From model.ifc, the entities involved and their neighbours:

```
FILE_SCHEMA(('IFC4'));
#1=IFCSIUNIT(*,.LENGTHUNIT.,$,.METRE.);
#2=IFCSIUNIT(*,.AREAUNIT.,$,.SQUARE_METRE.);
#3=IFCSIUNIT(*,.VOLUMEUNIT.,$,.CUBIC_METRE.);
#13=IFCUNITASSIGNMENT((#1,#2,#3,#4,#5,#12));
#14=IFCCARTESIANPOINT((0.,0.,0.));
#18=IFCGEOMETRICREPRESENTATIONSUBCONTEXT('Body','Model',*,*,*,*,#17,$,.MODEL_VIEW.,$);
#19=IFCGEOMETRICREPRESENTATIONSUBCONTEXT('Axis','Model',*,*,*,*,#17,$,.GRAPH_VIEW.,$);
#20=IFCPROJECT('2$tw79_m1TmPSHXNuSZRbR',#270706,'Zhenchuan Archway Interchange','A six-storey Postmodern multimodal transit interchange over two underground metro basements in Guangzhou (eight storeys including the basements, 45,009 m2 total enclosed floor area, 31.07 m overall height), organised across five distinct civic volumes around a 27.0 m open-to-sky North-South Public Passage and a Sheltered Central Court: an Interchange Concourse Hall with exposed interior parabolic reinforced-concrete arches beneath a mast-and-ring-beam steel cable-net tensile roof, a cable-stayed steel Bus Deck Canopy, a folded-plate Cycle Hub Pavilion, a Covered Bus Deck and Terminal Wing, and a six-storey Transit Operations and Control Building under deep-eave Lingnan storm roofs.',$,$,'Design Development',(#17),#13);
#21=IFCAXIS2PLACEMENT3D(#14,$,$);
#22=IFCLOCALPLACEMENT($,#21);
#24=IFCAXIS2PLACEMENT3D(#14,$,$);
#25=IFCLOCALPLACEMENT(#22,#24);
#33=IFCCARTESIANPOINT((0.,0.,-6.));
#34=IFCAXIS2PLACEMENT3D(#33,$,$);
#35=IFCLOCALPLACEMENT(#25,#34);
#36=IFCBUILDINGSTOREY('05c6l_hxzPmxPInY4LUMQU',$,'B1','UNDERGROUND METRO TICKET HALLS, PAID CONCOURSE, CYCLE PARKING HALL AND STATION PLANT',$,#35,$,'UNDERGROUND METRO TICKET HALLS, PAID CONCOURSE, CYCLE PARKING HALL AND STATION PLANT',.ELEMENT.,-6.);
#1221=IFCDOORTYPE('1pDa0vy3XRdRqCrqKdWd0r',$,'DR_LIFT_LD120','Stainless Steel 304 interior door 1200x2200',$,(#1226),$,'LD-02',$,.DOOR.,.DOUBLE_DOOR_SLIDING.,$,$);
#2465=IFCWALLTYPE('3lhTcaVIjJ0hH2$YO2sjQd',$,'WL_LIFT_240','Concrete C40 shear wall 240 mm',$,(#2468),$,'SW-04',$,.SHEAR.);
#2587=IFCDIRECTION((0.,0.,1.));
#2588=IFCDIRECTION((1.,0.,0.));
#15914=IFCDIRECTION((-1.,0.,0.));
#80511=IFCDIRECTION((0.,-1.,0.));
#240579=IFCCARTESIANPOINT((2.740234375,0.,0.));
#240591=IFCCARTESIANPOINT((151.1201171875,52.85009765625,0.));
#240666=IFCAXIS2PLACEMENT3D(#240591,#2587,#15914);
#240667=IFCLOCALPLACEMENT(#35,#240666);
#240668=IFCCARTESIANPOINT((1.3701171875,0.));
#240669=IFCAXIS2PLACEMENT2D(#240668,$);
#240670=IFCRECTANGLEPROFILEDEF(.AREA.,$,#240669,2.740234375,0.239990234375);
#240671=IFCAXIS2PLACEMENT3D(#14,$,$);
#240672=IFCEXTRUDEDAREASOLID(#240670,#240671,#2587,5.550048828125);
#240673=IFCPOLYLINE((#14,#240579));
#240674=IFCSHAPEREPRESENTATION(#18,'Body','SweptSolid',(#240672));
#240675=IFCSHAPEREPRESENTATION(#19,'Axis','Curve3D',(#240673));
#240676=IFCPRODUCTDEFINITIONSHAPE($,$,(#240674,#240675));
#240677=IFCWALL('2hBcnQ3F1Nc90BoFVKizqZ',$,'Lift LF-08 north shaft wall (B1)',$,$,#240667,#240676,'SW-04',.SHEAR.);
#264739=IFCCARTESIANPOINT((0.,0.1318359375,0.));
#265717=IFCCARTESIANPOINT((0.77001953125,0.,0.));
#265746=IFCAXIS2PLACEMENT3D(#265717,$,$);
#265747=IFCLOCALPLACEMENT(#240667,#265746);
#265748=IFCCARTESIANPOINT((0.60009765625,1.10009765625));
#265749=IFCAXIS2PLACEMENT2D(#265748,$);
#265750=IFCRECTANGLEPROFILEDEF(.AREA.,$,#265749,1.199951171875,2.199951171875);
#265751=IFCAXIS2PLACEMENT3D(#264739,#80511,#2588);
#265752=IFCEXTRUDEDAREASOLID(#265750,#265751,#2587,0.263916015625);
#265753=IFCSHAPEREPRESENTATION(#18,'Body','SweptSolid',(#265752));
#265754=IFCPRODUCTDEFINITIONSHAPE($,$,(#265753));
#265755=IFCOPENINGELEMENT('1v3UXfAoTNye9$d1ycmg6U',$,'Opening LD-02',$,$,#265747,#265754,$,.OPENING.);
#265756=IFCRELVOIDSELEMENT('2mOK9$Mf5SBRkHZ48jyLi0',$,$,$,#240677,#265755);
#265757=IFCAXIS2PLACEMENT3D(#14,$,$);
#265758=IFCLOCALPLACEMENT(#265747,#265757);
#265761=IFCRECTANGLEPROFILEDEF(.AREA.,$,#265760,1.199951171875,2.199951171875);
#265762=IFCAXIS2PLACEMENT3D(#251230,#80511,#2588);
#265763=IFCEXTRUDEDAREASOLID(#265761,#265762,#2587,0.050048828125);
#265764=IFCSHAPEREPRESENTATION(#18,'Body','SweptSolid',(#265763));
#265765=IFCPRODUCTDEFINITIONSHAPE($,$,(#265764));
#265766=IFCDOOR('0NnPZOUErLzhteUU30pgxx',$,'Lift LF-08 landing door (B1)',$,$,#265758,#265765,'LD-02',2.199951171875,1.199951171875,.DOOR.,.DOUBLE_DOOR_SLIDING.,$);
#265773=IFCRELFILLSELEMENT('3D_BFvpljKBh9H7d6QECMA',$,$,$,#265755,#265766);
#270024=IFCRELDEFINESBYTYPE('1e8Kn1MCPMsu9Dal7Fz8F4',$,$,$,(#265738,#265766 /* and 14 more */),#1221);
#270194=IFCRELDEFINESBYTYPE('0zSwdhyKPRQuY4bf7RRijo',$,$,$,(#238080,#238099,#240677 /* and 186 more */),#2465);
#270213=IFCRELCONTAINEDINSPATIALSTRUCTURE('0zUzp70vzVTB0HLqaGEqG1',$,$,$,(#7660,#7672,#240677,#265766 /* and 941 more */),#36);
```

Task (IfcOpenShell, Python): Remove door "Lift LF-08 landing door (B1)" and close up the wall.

```python
import ifcopenshell
import ifcopenshell.api.feature
import ifcopenshell.api.root
import ifcopenshell.geom
import ifcopenshell.util.shape

model = ifcopenshell.open("model.ifc")
settings = ifcopenshell.geom.settings()


def volume(element):
    """Net volume in cubic metres, openings subtracted."""
    shape = ifcopenshell.geom.create_shape(settings, element)
    return ifcopenshell.util.shape.get_volume(shape.geometry)


door = model.by_id(265766)
opening = door.FillsVoids[0].RelatingOpeningElement
wall = opening.VoidsElements[0].RelatingBuildingElement
before = volume(wall)

ifcopenshell.api.root.remove_product(model, product=door)
ifcopenshell.api.feature.remove_feature(model, feature=opening)

after = volume(wall)

print(f"wall volume {before:.3f} -> {after:.3f} m3")

model.write("model_updated.ifc")
```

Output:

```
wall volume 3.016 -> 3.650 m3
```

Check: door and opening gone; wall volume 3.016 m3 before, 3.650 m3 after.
